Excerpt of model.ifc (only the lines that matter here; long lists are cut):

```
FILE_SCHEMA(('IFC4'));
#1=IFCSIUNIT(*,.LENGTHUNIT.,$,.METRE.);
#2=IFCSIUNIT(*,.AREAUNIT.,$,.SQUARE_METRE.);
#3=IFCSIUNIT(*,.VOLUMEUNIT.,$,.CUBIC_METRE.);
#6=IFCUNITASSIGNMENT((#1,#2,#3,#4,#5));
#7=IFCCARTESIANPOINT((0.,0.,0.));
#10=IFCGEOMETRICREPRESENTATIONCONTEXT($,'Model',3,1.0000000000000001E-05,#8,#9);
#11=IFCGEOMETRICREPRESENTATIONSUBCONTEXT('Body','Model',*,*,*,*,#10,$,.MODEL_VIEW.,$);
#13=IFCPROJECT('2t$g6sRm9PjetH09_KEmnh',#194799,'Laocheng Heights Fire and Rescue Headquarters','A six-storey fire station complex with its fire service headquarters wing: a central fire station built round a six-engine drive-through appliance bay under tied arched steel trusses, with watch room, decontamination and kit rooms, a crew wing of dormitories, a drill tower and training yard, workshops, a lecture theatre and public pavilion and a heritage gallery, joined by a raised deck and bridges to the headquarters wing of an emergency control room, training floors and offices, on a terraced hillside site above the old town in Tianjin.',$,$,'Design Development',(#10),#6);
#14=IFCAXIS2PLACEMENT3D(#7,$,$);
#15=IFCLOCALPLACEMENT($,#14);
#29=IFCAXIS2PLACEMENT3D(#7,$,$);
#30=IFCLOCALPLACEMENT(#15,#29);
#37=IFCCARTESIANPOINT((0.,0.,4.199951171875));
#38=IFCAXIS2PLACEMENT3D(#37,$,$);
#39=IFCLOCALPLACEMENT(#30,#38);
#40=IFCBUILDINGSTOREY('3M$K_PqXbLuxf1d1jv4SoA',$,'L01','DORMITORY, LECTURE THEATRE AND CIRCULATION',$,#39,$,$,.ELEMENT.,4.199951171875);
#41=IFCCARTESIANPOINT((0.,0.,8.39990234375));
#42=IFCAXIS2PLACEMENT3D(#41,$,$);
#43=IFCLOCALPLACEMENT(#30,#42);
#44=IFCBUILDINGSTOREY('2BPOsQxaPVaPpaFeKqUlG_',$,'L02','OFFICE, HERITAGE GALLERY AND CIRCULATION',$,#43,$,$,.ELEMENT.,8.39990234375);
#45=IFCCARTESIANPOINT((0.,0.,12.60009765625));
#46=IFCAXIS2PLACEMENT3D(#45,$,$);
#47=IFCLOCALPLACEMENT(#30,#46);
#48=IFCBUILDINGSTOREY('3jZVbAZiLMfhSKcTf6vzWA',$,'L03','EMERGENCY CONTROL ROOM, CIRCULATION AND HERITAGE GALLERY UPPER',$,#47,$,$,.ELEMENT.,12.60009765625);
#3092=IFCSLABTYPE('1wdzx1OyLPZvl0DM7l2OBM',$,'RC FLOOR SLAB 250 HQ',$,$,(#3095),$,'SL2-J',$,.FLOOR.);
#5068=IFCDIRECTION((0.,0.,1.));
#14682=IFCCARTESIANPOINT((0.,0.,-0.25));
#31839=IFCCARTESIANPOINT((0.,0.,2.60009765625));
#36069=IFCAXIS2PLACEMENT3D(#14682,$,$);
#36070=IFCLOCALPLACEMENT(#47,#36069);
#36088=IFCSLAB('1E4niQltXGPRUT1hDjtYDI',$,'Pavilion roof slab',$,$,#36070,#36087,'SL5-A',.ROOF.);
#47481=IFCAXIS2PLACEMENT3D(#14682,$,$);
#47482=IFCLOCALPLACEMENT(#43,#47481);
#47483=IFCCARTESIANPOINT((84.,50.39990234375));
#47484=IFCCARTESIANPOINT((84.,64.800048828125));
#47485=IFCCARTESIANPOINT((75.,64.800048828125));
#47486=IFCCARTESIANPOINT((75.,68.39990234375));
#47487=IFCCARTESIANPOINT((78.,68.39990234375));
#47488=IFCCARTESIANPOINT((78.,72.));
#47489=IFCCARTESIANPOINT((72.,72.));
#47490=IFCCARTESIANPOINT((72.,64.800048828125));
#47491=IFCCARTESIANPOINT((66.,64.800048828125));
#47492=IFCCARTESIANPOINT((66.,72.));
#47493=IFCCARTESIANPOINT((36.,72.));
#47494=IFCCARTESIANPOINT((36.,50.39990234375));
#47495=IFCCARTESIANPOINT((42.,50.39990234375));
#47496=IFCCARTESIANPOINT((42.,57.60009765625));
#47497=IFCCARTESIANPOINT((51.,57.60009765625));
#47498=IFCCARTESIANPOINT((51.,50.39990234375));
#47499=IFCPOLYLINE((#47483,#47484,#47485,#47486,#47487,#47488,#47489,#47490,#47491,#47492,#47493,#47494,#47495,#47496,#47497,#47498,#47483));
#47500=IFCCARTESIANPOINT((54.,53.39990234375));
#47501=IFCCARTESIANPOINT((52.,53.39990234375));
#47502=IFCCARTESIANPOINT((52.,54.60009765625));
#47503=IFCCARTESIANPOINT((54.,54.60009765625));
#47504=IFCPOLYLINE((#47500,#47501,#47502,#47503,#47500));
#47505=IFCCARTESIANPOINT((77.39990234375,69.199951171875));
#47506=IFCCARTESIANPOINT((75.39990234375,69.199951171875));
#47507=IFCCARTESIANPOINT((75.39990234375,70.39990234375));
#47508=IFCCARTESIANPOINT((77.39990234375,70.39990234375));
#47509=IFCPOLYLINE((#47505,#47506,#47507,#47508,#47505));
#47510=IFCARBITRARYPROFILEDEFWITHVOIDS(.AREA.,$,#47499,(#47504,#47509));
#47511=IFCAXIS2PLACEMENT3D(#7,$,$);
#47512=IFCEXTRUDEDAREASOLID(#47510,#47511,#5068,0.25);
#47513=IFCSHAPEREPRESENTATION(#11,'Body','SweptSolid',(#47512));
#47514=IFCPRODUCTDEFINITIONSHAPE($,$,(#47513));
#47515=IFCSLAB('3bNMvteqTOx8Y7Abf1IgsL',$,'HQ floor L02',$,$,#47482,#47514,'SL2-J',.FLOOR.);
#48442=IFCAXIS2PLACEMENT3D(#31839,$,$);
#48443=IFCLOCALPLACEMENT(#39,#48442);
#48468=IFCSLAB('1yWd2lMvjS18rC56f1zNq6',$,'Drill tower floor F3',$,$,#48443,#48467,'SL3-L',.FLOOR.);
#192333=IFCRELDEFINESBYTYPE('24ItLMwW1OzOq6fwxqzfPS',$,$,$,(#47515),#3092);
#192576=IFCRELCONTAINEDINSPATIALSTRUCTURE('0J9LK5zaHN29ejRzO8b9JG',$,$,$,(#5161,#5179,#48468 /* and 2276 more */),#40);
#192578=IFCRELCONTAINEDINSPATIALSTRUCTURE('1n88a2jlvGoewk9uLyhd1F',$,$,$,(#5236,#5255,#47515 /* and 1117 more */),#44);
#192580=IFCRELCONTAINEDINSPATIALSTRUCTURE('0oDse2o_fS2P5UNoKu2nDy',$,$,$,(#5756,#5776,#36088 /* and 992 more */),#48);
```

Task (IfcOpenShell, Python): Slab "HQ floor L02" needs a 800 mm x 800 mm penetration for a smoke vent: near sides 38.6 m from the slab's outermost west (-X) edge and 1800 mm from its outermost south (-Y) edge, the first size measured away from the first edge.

```python
import numpy as np
import ifcopenshell
import ifcopenshell.api.feature
import ifcopenshell.api.geometry
import ifcopenshell.api.root
import ifcopenshell.geom
import ifcopenshell.util.placement
import ifcopenshell.util.representation
import ifcopenshell.util.shape
import ifcopenshell.util.unit

model = ifcopenshell.open("model.ifc")
unit_scale = ifcopenshell.util.unit.calculate_unit_scale(model)
settings = ifcopenshell.geom.settings()


def volume(element):
    """Net volume in cubic metres, openings subtracted."""
    shape = ifcopenshell.geom.create_shape(settings, element)
    return ifcopenshell.util.shape.get_volume(shape.geometry)


slab = model.by_id(47515)
before = volume(slab)

# Extent in the slab's own axes, in metres. The edges named are its -X and -Y sides.
slab_shape = ifcopenshell.geom.create_shape(settings, slab)
vertices = ifcopenshell.util.shape.get_vertices(slab_shape.geometry)
x_min, y_min, bottom = vertices.min(axis=0)
top = vertices[:, 2].max()

opening = ifcopenshell.api.root.create_entity(model, ifc_class="IfcOpeningElement", name="Smoke vent opening", predefined_type="OPENING")
context = ifcopenshell.util.representation.get_context(model, "Model", "Body", "MODEL_VIEW")
width, depth = 0.8, 0.8
outline = [(0.0, 0.0), (width, 0.0), (width, depth), (0.0, depth), (0.0, 0.0)]
# Overshoot both faces by 50 mm so the cut is clean.
shape = ifcopenshell.api.geometry.add_slab_representation(
    model, context=context, depth=top - bottom + 0.1, polyline=outline
)
ifcopenshell.api.geometry.assign_representation(model, product=opening, representation=shape)

matrix = ifcopenshell.util.placement.get_local_placement(slab.ObjectPlacement)
matrix[:, 3] = matrix @ np.append(np.array([x_min + 38.6, y_min + 1.8, bottom - 0.05]) / unit_scale, 1.0)
ifcopenshell.api.geometry.edit_object_placement(model, product=opening, matrix=matrix, is_si=False)
ifcopenshell.api.feature.add_feature(model, feature=opening, element=slab)

after = volume(slab)

print(f"slab volume {before:.3f} -> {after:.3f} m3")

model.write("model_updated.ifc")
```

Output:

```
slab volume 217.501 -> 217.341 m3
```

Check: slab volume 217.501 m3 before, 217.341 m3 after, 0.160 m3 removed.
